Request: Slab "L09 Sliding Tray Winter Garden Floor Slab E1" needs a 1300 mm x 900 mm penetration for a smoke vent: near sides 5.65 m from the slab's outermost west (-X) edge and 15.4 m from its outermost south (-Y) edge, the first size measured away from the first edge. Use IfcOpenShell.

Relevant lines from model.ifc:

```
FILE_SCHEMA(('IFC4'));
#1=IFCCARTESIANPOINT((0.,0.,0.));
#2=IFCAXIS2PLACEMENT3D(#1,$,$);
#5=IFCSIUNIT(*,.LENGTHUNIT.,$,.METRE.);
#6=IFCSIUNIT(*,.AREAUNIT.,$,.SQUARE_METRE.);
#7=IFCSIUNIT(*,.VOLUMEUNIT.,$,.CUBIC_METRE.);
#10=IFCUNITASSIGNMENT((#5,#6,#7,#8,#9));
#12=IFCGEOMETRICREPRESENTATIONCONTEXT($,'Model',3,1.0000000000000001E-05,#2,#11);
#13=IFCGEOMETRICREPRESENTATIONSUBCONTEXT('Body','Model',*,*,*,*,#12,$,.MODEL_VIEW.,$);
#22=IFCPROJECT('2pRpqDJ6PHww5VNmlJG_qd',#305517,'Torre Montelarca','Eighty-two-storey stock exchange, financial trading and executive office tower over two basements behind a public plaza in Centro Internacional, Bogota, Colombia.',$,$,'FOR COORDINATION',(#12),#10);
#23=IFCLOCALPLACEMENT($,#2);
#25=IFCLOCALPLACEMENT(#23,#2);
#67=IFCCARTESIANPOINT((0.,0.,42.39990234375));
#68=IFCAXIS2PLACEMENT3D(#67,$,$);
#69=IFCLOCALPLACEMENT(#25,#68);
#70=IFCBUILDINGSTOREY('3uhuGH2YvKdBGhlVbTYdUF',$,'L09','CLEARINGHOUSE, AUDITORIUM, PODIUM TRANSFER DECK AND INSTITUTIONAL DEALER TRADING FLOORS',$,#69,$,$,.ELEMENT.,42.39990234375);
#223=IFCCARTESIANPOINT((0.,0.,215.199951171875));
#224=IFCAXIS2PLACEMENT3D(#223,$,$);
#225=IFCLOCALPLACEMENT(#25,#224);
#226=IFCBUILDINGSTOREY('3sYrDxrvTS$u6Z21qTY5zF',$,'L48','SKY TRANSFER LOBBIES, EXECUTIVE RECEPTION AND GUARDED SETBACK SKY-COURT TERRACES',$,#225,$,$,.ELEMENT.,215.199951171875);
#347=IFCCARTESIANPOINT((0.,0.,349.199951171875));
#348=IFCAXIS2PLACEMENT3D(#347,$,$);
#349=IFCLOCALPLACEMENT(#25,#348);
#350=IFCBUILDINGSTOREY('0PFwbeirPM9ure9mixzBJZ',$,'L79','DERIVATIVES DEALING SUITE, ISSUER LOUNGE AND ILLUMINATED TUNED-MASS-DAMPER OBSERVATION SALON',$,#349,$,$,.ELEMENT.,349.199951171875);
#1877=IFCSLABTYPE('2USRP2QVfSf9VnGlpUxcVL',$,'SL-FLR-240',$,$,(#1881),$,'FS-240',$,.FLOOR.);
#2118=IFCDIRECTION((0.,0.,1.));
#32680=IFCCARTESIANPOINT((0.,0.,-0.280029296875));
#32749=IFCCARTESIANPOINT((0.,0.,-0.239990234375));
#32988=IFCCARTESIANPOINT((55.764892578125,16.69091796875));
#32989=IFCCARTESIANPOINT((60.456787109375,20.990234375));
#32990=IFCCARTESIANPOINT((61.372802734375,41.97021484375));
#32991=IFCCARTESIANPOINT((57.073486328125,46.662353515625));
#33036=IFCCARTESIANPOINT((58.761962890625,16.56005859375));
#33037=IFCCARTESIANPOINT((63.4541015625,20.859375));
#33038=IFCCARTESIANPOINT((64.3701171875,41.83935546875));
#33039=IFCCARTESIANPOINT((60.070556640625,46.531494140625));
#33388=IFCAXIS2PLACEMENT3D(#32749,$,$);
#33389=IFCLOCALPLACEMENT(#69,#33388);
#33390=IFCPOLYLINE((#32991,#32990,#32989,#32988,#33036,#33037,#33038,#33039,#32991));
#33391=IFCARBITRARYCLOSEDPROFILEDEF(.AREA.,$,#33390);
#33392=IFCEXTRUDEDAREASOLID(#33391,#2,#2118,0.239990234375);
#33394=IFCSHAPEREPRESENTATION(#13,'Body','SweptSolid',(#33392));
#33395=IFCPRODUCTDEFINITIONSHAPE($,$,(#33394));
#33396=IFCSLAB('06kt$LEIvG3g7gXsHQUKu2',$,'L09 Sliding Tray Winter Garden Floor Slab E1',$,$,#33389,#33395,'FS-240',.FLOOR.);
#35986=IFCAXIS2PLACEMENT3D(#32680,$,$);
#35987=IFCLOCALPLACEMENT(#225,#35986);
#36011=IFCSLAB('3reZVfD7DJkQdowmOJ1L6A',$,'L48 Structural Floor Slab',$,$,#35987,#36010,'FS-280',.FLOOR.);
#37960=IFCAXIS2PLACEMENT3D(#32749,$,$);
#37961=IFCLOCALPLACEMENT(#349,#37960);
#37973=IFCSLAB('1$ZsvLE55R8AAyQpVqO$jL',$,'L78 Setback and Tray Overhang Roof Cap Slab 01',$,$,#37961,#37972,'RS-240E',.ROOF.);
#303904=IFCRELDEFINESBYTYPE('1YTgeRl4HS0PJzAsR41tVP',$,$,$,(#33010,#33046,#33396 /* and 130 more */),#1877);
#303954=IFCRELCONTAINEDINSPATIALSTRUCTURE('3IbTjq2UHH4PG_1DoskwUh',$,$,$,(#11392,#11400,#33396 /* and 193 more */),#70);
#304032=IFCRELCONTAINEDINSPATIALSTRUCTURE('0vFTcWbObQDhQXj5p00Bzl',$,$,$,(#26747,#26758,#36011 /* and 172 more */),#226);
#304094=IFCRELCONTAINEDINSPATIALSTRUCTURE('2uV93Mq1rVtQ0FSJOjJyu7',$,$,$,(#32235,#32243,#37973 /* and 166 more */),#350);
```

```python
import numpy as np
import ifcopenshell
import ifcopenshell.api.feature
import ifcopenshell.api.geometry
import ifcopenshell.api.root
import ifcopenshell.geom
import ifcopenshell.util.placement
import ifcopenshell.util.representation
import ifcopenshell.util.shape
import ifcopenshell.util.unit

model = ifcopenshell.open("model.ifc")
unit_scale = ifcopenshell.util.unit.calculate_unit_scale(model)
settings = ifcopenshell.geom.settings()


def volume(element):
    """Net volume in cubic metres, openings subtracted."""
    shape = ifcopenshell.geom.create_shape(settings, element)
    return ifcopenshell.util.shape.get_volume(shape.geometry)


slab = model.by_guid("06kt$LEIvG3g7gXsHQUKu2")
before = volume(slab)

# Extent in the slab's own axes, in metres. The edges named are its -X and -Y sides.
slab_shape = ifcopenshell.geom.create_shape(settings, slab)
vertices = ifcopenshell.util.shape.get_vertices(slab_shape.geometry)
x_min, y_min, bottom = vertices.min(axis=0)
top = vertices[:, 2].max()

opening = ifcopenshell.api.root.create_entity(model, ifc_class="IfcOpeningElement", name="Smoke vent opening", predefined_type="OPENING")
context = ifcopenshell.util.representation.get_context(model, "Model", "Body", "MODEL_VIEW")
width, depth = 1.3, 0.9
outline = [(0.0, 0.0), (width, 0.0), (width, depth), (0.0, depth), (0.0, 0.0)]
# Overshoot both faces by 50 mm so the cut is clean.
shape = ifcopenshell.api.geometry.add_slab_representation(
    model, context=context, depth=top - bottom + 0.1, polyline=outline
)
ifcopenshell.api.geometry.assign_representation(model, product=opening, representation=shape)

matrix = ifcopenshell.util.placement.get_local_placement(slab.ObjectPlacement)
matrix[:, 3] = matrix @ np.append(np.array([x_min + 5.65, y_min + 15.4, bottom - 0.05]) / unit_scale, 1.0)
ifcopenshell.api.geometry.edit_object_placement(model, product=opening, matrix=matrix, is_si=False)
ifcopenshell.api.feature.add_feature(model, feature=opening, element=slab)

after = volume(slab)

print(f"slab volume {before:.3f} -> {after:.3f} m3")

model.write("model_edited.ifc")
```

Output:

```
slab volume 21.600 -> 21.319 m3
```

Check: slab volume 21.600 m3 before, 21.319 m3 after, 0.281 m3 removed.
